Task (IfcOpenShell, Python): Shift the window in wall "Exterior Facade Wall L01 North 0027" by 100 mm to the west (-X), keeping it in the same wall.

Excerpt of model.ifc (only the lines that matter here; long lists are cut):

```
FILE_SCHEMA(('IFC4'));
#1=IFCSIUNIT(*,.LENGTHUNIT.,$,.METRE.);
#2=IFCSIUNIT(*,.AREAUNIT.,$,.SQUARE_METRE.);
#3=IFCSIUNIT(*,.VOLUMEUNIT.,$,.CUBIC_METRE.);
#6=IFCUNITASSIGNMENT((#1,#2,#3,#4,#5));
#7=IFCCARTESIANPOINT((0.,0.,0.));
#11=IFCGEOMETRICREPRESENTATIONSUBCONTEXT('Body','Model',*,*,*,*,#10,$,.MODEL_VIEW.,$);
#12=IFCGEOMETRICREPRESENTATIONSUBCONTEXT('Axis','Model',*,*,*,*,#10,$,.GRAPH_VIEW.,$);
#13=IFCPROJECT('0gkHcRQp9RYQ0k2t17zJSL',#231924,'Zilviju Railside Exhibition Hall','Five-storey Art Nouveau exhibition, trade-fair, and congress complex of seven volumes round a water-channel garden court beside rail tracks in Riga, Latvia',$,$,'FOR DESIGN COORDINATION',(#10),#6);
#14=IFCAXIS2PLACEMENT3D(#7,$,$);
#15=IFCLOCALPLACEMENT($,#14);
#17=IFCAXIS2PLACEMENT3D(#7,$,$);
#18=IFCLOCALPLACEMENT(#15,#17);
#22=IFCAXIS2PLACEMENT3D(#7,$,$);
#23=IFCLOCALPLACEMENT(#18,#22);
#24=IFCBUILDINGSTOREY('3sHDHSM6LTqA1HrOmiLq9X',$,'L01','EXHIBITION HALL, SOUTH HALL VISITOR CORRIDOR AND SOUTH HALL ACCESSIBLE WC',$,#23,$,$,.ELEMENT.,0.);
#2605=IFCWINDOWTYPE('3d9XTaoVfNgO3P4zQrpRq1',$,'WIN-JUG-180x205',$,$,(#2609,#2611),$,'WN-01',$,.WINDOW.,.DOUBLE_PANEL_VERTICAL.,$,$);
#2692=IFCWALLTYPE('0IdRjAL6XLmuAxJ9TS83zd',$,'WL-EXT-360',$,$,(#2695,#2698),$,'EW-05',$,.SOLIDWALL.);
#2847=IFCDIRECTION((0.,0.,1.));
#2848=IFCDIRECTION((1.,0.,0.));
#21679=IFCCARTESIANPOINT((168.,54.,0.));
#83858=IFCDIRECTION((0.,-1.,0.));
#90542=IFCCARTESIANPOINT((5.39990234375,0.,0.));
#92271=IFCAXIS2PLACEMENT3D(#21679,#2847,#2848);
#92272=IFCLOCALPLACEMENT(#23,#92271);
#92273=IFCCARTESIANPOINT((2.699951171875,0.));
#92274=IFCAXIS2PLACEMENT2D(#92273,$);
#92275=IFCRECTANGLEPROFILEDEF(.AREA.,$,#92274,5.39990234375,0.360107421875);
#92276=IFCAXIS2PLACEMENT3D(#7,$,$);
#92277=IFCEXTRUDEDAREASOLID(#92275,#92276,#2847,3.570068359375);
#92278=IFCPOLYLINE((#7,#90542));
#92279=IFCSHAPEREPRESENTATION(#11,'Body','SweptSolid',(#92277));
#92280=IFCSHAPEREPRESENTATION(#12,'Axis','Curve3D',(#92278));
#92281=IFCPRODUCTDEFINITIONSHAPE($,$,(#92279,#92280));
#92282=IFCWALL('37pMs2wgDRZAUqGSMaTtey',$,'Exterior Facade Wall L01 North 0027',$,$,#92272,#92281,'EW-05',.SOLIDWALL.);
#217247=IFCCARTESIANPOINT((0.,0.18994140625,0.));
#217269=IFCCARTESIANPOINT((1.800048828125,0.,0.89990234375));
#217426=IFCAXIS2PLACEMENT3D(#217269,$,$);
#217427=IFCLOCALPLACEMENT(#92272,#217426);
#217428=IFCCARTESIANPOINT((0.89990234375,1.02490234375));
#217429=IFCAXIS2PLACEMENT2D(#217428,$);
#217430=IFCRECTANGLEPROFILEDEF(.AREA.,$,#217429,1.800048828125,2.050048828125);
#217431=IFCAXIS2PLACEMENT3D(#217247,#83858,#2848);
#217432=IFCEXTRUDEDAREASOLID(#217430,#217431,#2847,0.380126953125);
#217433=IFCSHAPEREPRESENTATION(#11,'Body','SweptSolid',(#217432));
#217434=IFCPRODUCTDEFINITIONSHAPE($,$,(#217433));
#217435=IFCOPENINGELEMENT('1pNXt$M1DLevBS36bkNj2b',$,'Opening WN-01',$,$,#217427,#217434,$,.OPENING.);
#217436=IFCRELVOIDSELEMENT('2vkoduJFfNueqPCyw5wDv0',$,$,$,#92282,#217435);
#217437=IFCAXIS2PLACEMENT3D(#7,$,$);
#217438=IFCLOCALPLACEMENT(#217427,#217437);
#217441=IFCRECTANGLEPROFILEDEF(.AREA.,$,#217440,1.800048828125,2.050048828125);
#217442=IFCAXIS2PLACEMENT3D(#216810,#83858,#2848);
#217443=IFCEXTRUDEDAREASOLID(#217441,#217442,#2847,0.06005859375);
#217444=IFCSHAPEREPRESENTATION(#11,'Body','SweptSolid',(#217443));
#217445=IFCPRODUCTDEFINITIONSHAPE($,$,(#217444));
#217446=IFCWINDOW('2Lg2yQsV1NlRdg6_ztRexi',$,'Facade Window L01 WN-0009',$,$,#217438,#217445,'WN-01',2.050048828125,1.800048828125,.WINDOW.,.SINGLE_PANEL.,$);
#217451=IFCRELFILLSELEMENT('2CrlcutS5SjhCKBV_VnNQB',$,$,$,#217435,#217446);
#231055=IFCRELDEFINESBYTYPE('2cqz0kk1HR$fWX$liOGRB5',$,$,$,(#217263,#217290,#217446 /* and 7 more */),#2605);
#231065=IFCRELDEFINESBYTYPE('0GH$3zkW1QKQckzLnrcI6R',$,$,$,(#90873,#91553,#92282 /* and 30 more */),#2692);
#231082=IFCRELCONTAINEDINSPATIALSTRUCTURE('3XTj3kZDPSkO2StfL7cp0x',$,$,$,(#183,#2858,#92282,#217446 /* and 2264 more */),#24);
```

```python
import ifcopenshell
import ifcopenshell.api.geometry
import ifcopenshell.util.placement
import ifcopenshell.util.unit

model = ifcopenshell.open("model.ifc")
unit_scale = ifcopenshell.util.unit.calculate_unit_scale(model)

window = model.by_guid("2Lg2yQsV1NlRdg6_ztRexi")
opening = window.FillsVoids[0].RelatingOpeningElement
wall = opening.VoidsElements[0].RelatingBuildingElement

wall_matrix = ifcopenshell.util.placement.get_local_placement(wall.ObjectPlacement)
shift = wall_matrix[:3, 0] * -0.1 / unit_scale
before = ifcopenshell.util.placement.get_local_placement(window.ObjectPlacement)[:3, 3].copy()

# The window is placed relative to its opening, so it follows when the opening moves.
matrix = ifcopenshell.util.placement.get_local_placement(opening.ObjectPlacement)
matrix[:3, 3] += shift
ifcopenshell.api.geometry.edit_object_placement(
    model, product=opening, matrix=matrix, is_si=False, should_transform_children=True
)

after = ifcopenshell.util.placement.get_local_placement(window.ObjectPlacement)[:3, 3]
print("window moved by", (after - before).round(3) + 0.0)

model.write("model_rev.ifc")
```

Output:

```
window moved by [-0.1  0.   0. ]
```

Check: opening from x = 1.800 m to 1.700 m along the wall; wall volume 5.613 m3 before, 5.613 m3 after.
